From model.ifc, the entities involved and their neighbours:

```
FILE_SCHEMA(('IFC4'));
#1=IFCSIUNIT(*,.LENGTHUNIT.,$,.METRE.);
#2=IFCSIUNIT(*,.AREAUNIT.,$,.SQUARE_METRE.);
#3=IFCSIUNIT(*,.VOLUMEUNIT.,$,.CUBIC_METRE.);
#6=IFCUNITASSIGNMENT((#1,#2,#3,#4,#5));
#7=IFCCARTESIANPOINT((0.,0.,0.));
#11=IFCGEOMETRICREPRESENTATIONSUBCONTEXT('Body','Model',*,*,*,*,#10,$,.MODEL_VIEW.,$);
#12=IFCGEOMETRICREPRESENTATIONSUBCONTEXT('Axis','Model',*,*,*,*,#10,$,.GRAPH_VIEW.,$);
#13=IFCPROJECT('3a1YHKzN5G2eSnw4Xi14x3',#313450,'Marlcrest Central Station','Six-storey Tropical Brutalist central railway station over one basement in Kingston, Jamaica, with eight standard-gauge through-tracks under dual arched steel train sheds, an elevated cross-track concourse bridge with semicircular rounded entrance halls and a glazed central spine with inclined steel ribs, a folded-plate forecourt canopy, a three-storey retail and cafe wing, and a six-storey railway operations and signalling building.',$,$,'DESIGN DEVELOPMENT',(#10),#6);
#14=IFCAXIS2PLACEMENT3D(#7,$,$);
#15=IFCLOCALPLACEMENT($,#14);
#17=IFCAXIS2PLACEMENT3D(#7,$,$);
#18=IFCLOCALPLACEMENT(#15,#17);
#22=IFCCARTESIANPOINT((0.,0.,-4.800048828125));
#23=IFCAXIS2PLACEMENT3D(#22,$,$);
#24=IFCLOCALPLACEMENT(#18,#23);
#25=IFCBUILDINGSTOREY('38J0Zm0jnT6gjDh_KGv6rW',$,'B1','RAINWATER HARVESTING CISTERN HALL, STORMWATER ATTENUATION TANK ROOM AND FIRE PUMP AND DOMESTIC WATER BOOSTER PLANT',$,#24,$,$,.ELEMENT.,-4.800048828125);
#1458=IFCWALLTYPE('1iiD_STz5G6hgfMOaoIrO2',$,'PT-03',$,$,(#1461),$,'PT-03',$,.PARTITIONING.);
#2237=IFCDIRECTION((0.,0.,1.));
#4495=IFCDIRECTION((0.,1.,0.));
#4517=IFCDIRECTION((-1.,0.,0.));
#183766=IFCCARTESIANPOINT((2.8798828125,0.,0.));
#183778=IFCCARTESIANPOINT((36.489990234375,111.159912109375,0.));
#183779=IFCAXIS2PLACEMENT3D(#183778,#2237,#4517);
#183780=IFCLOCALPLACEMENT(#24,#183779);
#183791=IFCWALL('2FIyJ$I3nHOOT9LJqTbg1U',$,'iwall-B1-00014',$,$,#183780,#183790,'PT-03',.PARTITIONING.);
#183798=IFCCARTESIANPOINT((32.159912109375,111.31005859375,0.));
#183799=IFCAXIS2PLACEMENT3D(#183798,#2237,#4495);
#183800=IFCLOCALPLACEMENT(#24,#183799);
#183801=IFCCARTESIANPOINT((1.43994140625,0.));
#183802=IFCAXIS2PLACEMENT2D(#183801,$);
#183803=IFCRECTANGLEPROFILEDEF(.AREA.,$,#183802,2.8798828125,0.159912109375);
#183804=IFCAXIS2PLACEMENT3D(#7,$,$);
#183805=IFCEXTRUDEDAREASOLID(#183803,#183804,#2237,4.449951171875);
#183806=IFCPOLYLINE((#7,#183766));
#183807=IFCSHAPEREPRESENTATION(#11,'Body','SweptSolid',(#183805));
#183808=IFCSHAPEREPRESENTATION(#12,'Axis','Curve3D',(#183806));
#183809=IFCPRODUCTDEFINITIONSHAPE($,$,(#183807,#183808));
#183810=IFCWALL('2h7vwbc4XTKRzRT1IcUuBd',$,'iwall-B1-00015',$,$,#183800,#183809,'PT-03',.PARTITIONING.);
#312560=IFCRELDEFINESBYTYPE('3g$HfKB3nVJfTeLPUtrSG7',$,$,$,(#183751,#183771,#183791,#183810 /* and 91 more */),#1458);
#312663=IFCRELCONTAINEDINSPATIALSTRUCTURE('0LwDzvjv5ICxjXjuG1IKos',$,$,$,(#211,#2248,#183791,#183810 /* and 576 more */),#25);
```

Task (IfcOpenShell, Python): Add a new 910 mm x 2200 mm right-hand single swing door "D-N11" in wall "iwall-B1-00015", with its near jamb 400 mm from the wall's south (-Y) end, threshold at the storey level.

```python
import numpy as np
import ifcopenshell
import ifcopenshell.api.feature
import ifcopenshell.api.geometry
import ifcopenshell.api.root
import ifcopenshell.api.spatial
import ifcopenshell.geom
import ifcopenshell.util.element
import ifcopenshell.util.placement
import ifcopenshell.util.representation
import ifcopenshell.util.shape
import ifcopenshell.util.unit

model = ifcopenshell.open("model.ifc")
unit_scale = ifcopenshell.util.unit.calculate_unit_scale(model)
settings = ifcopenshell.geom.settings()


def volume(element):
    """Net volume in cubic metres, openings subtracted."""
    shape = ifcopenshell.geom.create_shape(settings, element)
    return ifcopenshell.util.shape.get_volume(shape.geometry)


wall = model.by_guid("2h7vwbc4XTKRzRT1IcUuBd")
storey = ifcopenshell.util.element.get_container(wall, ifc_class="IfcBuildingStorey")
context = ifcopenshell.util.representation.get_context(model, "Model", "Body", "MODEL_VIEW")
before = volume(wall)

width, height, from_end, sill = 0.91, 2.2, 0.4, 0.0  # metres

# The wall runs along its own X axis, and the end named is its -X end.
wall_shape = ifcopenshell.geom.create_shape(settings, wall)
x, y, z = ifcopenshell.util.shape.get_vertices(wall_shape.geometry).T
start = x.min() + from_end
face, thickness = float(y.min()), float(y.max() - y.min())
wall_matrix = ifcopenshell.util.placement.get_local_placement(wall.ObjectPlacement)
level = ifcopenshell.util.placement.get_local_placement(storey.ObjectPlacement)[2, 3]


def in_wall(x, y):
    """Placement at x, y metres in the wall's axes, at sill height."""
    matrix = wall_matrix.copy()
    matrix[:, 3] = wall_matrix @ np.array([x / unit_scale, y / unit_scale, 0.0, 1.0])
    matrix[2, 3] = level + sill / unit_scale
    return matrix


# Opening: a box that overshoots both wall faces by 50 mm.
opening = ifcopenshell.api.root.create_entity(model, ifc_class="IfcOpeningElement", predefined_type="OPENING")
box = ifcopenshell.api.geometry.add_wall_representation(
    model, context=context, length=width, height=height, thickness=thickness + 0.1
)
ifcopenshell.api.geometry.assign_representation(model, product=opening, representation=box)
ifcopenshell.api.geometry.edit_object_placement(model, product=opening, matrix=in_wall(start, face - 0.05), is_si=False)
ifcopenshell.api.feature.add_feature(model, feature=opening, element=wall)

door = ifcopenshell.api.root.create_entity(model, ifc_class="IfcDoor", name="D-N11", predefined_type="DOOR")
door.OverallWidth, door.OverallHeight = width / unit_scale, height / unit_scale
door.OperationType = "SINGLE_SWING_RIGHT"
body = ifcopenshell.api.geometry.add_door_representation(
    model,
    context=context,
    overall_width=door.OverallWidth,
    overall_height=door.OverallHeight,
    operation_type="SINGLE_SWING_RIGHT",
    lining_properties={"LiningDepth": thickness / unit_scale, "ThresholdDepth": thickness / unit_scale},
)
ifcopenshell.api.geometry.assign_representation(model, product=door, representation=body)
ifcopenshell.api.spatial.assign_container(model, products=[door], relating_structure=storey)
ifcopenshell.api.feature.add_filling(model, opening=opening, element=door)

# The lining spans the wall, so the door starts at the wall face.
ifcopenshell.api.geometry.edit_object_placement(model, product=door, matrix=in_wall(start, face), is_si=False)

after = volume(wall)

print(f"wall volume {before:.3f} -> {after:.3f} m3")

model.write("model_rev.ifc")
```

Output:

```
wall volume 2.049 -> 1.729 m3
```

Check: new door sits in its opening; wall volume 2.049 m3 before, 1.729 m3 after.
